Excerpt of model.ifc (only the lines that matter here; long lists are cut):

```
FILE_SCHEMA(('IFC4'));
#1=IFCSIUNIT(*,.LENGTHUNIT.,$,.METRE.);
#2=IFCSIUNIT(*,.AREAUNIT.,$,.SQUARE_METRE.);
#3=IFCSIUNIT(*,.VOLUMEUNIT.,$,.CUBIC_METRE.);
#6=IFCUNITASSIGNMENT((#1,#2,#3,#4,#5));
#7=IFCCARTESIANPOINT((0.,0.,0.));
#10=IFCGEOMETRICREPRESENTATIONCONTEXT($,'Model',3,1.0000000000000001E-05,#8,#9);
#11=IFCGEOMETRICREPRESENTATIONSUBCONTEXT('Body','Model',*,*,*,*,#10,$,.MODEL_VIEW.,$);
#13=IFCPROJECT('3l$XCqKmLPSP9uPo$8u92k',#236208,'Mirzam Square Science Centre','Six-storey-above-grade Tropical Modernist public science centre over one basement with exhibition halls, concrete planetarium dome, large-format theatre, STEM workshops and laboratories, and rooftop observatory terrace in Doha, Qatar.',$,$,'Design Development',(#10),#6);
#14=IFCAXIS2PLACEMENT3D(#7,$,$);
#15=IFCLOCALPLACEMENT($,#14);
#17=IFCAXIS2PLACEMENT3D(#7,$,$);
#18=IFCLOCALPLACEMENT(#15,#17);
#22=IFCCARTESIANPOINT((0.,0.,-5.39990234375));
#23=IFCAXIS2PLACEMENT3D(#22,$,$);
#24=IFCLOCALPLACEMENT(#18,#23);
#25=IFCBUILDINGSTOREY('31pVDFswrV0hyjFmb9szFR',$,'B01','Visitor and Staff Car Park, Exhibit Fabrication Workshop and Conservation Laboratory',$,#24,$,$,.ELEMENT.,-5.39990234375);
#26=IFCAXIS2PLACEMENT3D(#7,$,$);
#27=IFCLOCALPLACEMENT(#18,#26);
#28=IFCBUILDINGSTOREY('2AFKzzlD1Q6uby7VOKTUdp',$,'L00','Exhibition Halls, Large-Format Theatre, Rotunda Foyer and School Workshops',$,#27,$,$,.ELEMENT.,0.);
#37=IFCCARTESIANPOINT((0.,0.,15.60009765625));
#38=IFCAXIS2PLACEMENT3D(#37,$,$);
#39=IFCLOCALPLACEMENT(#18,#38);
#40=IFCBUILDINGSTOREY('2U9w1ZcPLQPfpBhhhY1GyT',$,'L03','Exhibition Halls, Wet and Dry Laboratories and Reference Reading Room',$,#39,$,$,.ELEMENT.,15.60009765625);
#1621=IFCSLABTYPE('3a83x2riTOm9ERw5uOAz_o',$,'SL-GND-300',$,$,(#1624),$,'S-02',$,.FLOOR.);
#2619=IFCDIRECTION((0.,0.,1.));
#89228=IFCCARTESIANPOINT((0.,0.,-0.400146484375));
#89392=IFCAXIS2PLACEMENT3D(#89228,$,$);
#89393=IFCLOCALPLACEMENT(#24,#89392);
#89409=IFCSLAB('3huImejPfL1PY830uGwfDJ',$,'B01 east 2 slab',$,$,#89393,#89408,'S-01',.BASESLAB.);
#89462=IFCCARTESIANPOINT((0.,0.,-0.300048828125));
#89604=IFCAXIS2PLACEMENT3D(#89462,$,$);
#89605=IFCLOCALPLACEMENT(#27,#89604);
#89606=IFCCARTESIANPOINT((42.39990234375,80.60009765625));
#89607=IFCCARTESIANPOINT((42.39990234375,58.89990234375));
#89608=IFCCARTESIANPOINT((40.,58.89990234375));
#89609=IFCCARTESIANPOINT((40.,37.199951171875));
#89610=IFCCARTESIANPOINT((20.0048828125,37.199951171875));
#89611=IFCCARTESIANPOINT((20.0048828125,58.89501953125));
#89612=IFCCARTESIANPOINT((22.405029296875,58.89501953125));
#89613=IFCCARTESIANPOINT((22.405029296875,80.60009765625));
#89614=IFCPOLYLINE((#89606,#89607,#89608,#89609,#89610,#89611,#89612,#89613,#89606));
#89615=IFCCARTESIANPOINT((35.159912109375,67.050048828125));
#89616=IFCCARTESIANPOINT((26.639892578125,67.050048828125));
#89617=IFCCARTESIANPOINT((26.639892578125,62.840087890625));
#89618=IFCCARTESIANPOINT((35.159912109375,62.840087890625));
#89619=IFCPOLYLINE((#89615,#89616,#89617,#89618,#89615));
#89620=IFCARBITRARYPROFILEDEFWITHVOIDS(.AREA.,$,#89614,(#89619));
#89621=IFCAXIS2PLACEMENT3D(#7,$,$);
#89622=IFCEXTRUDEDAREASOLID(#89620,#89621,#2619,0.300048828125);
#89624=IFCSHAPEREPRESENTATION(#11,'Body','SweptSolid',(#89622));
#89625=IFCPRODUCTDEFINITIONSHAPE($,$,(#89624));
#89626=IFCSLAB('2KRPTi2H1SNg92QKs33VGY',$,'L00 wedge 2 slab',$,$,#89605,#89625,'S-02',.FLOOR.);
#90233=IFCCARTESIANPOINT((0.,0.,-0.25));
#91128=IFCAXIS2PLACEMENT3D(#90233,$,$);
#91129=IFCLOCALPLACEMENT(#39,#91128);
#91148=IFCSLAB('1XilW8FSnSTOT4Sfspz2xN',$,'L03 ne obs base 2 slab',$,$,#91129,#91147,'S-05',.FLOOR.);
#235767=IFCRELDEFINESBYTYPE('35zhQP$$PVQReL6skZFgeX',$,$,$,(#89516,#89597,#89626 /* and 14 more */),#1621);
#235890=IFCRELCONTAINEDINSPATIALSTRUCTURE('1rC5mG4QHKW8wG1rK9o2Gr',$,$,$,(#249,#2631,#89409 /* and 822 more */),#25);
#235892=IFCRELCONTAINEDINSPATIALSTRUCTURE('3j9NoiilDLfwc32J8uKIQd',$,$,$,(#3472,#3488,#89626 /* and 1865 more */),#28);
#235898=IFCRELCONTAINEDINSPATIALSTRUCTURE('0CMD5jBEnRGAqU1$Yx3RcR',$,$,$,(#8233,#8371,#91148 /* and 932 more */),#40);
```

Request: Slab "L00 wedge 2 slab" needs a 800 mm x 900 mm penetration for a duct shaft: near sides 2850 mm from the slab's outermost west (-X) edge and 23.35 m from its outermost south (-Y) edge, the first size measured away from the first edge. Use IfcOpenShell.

```python
import numpy as np
import ifcopenshell
import ifcopenshell.api.feature
import ifcopenshell.api.geometry
import ifcopenshell.api.root
import ifcopenshell.geom
import ifcopenshell.util.placement
import ifcopenshell.util.representation
import ifcopenshell.util.shape
import ifcopenshell.util.unit

model = ifcopenshell.open("model.ifc")
unit_scale = ifcopenshell.util.unit.calculate_unit_scale(model)
settings = ifcopenshell.geom.settings()


def volume(element):
    """Net volume in cubic metres, openings subtracted."""
    shape = ifcopenshell.geom.create_shape(settings, element)
    return ifcopenshell.util.shape.get_volume(shape.geometry)


slab = model.by_id(89626)
before = volume(slab)

# Extent in the slab's own axes, in metres. The edges named are its -X and -Y sides.
slab_shape = ifcopenshell.geom.create_shape(settings, slab)
vertices = ifcopenshell.util.shape.get_vertices(slab_shape.geometry)
x_min, y_min, bottom = vertices.min(axis=0)
top = vertices[:, 2].max()

opening = ifcopenshell.api.root.create_entity(model, ifc_class="IfcOpeningElement", name="Duct shaft opening", predefined_type="OPENING")
context = ifcopenshell.util.representation.get_context(model, "Model", "Body", "MODEL_VIEW")
width, depth = 0.8, 0.9
outline = [(0.0, 0.0), (width, 0.0), (width, depth), (0.0, depth), (0.0, 0.0)]
# Overshoot both faces by 50 mm so the cut is clean.
shape = ifcopenshell.api.geometry.add_slab_representation(
    model, context=context, depth=top - bottom + 0.1, polyline=outline
)
ifcopenshell.api.geometry.assign_representation(model, product=opening, representation=shape)

matrix = ifcopenshell.util.placement.get_local_placement(slab.ObjectPlacement)
matrix[:, 3] = matrix @ np.append(np.array([x_min + 2.85, y_min + 23.35, bottom - 0.05]) / unit_scale, 1.0)
ifcopenshell.api.geometry.edit_object_placement(model, product=opening, matrix=matrix, is_si=False)
ifcopenshell.api.feature.add_feature(model, feature=opening, element=slab)

after = volume(slab)

print(f"slab volume {before:.3f} -> {after:.3f} m3")

model.write("model_v2.ifc")
```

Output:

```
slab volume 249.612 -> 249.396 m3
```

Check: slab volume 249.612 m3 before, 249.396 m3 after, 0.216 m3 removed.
